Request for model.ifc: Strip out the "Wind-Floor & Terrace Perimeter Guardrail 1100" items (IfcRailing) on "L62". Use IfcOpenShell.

First a look at what the model holds.

```python
import ifcopenshell
import ifcopenshell.util.element

model = ifcopenshell.open("model.ifc")
print(model.schema)
storey = next(s for s in model.by_type("IfcBuildingStorey") if s.Name == "L62")
railings = [e for e in ifcopenshell.util.element.get_decomposition(storey) if e.is_a("IfcRailing")]
seen = {}
for e in railings:
    element_type = ifcopenshell.util.element.get_type(e)
    name = element_type.Name if element_type not in (None, e) else None
    seen[name] = seen.get(name, 0) + 1
for name, count in sorted(seen.items(), key=str):
    print(count, "x", name)
```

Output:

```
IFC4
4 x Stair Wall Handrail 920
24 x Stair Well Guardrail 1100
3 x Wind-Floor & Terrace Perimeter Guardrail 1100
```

```python
import ifcopenshell
import ifcopenshell.api.root
import ifcopenshell.util.element

model = ifcopenshell.open("model.ifc")

storey = next(s for s in model.by_type("IfcBuildingStorey") if s.Name == "L62")
railings = [e for e in ifcopenshell.util.element.get_decomposition(storey) if e.is_a("IfcRailing")]
targets = [e for e in railings if (t := ifcopenshell.util.element.get_type(e)) not in (None, e) and t.Name == "Wind-Floor & Terrace Perimeter Guardrail 1100"]

for e in targets:
    ifcopenshell.api.root.remove_product(model, product=e)
print(len(targets), "removed")

model.write("model_v2.ifc")
```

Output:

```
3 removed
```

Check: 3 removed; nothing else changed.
